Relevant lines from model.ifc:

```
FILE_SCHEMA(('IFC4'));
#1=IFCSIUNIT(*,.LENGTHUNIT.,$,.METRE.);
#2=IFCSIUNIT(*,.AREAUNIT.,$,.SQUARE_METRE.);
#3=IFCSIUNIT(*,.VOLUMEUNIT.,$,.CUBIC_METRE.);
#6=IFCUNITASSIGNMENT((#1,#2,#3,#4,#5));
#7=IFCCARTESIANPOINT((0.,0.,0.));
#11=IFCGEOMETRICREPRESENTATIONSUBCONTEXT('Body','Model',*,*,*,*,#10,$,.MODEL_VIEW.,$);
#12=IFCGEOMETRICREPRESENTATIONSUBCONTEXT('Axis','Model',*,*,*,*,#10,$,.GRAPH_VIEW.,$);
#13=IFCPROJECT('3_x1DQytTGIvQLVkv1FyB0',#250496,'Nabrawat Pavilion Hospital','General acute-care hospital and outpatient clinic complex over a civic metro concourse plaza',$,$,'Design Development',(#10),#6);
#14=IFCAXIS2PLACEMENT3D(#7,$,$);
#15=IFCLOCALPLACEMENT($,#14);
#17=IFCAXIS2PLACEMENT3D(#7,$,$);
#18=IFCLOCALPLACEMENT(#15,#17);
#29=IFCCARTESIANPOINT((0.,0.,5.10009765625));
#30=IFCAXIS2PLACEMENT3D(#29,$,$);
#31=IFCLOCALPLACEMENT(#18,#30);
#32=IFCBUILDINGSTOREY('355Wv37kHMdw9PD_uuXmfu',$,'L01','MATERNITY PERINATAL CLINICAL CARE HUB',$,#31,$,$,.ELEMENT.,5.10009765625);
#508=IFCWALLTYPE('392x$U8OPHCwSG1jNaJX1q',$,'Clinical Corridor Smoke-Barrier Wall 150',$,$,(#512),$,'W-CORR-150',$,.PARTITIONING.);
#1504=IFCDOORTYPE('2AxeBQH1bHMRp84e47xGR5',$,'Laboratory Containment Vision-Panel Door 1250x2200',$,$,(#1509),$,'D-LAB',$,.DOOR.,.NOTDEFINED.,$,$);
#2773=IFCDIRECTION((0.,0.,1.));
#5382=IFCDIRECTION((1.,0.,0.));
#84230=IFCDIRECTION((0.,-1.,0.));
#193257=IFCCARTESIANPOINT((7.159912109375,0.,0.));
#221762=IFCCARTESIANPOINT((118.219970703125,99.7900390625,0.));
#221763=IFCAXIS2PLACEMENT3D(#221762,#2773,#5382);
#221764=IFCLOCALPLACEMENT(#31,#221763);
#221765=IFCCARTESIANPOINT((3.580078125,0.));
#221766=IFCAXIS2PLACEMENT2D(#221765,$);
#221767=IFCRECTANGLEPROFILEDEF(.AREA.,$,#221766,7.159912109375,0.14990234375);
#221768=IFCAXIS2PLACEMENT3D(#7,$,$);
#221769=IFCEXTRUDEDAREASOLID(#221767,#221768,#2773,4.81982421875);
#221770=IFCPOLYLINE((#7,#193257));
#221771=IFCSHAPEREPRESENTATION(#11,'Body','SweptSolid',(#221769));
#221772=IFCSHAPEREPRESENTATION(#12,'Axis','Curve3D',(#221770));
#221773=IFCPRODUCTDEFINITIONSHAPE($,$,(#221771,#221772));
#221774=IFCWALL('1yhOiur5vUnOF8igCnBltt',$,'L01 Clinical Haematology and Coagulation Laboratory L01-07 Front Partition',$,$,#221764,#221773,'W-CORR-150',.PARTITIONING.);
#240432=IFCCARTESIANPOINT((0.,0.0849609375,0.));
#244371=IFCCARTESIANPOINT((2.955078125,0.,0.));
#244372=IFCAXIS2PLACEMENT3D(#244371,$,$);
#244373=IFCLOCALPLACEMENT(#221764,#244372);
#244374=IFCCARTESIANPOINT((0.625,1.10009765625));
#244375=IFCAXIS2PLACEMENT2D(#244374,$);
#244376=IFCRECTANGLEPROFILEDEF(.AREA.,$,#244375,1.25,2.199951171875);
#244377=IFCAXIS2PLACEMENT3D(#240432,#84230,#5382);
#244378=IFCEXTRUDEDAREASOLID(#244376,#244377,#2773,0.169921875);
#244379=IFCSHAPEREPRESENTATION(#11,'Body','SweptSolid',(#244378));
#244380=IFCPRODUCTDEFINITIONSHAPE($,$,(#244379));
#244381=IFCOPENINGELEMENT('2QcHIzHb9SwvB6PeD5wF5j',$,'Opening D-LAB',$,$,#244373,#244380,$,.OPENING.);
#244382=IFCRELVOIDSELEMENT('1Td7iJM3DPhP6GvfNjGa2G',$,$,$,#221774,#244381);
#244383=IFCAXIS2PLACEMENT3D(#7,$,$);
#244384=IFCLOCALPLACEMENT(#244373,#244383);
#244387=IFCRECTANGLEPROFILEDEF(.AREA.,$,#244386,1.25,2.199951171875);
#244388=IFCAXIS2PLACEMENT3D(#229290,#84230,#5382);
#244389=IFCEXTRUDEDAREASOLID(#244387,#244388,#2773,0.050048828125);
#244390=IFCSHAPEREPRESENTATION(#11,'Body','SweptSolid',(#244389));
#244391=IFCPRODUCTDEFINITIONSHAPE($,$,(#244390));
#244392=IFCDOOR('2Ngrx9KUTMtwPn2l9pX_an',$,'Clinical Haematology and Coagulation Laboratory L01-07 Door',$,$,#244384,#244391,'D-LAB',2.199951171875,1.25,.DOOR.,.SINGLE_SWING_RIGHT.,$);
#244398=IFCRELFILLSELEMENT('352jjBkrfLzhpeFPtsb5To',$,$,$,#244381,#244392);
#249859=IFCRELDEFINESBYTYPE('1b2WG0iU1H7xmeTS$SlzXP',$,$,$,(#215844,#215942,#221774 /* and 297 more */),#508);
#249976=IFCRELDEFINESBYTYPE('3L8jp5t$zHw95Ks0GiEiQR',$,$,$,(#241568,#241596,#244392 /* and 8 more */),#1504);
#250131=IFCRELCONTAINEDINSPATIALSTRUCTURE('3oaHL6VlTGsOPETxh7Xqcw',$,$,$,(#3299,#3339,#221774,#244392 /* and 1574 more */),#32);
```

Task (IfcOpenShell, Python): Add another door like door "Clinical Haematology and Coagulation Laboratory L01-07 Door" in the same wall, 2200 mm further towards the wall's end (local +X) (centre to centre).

```python
import ifcopenshell
import ifcopenshell.api.feature
import ifcopenshell.api.geometry
import ifcopenshell.api.root
import ifcopenshell.geom
import ifcopenshell.util.element
import ifcopenshell.util.placement
import ifcopenshell.util.shape
import ifcopenshell.util.unit

model = ifcopenshell.open("model.ifc")
unit_scale = ifcopenshell.util.unit.calculate_unit_scale(model)
settings = ifcopenshell.geom.settings()


def volume(element):
    """Net volume in cubic metres, openings subtracted."""
    shape = ifcopenshell.geom.create_shape(settings, element)
    return ifcopenshell.util.shape.get_volume(shape.geometry)


door = model.by_guid("2Ngrx9KUTMtwPn2l9pX_an")
opening = door.FillsVoids[0].RelatingOpeningElement
wall = opening.VoidsElements[0].RelatingBuildingElement
before = volume(wall)
shift = ifcopenshell.util.placement.get_local_placement(wall.ObjectPlacement)[:3, 0] * 2.2 / unit_scale

# copy_class copies the void relationship, type, container and properties, but no geometry.
new_opening = ifcopenshell.api.root.copy_class(model, product=opening)
new_opening.Representation = ifcopenshell.util.element.copy_deep(
    model, opening.Representation, exclude=["IfcGeometricRepresentationContext", "IfcRepresentationMap"]
)
new_door = ifcopenshell.api.root.copy_class(model, product=door)
new_door.Representation = ifcopenshell.util.element.copy_deep(
    model, door.Representation, exclude=["IfcGeometricRepresentationContext", "IfcRepresentationMap"]
)
new_door.Tag = None
ifcopenshell.api.feature.add_filling(model, opening=new_opening, element=new_door)

for old, new in ((opening, new_opening), (door, new_door)):
    matrix = ifcopenshell.util.placement.get_local_placement(old.ObjectPlacement)
    matrix[:3, 3] += shift
    ifcopenshell.api.geometry.edit_object_placement(model, product=new, matrix=matrix, is_si=False)

after = volume(wall)

print(f"wall volume {before:.3f} -> {after:.3f} m3")

model.write("model_updated.ifc")
```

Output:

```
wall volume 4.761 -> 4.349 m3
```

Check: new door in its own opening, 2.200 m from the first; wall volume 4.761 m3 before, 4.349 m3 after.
